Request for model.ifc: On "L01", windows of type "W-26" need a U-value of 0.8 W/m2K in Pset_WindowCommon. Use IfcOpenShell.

First a look at what the model holds.

```python
import ifcopenshell
import ifcopenshell.util.element

model = ifcopenshell.open("model.ifc")
print(model.schema)
storey = next(s for s in model.by_type("IfcBuildingStorey") if s.Name == "L01")
windows = [e for e in ifcopenshell.util.element.get_decomposition(storey) if e.is_a("IfcWindow")]
seen = {}
for e in windows:
    element_type = ifcopenshell.util.element.get_type(e)
    key = (element_type.Name if element_type != e and element_type else None, ifcopenshell.util.element.get_pset(e, "Pset_WindowCommon", "ThermalTransmittance"))
    seen[key] = seen.get(key, 0) + 1
for (name, value), count in sorted(seen.items(), key=str):
    print(count, "x", name, "|", value)
```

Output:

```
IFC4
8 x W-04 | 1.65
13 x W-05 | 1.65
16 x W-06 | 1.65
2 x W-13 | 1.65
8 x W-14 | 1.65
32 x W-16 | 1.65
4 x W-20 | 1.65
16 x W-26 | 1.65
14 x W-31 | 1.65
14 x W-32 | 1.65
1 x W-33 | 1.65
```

```python
import ifcopenshell
import ifcopenshell.api.pset
import ifcopenshell.util.element

model = ifcopenshell.open("model.ifc")

storey = next(s for s in model.by_type("IfcBuildingStorey") if s.Name == "L01")
windows = [e for e in ifcopenshell.util.element.get_decomposition(storey) if e.is_a("IfcWindow")]

count = 0
for e in windows:
    element_type = ifcopenshell.util.element.get_type(e)
    if element_type in (None, e) or element_type.Name != "W-26":
        continue
    # add_pset returns the element's existing set when there is one.
    pset = ifcopenshell.api.pset.add_pset(model, product=e, name="Pset_WindowCommon")
    ifcopenshell.api.pset.edit_pset(model, pset=pset, properties={"ThermalTransmittance": 0.8})
    count += 1

print(count, "windows updated")

model.write("model_edited.ifc")
```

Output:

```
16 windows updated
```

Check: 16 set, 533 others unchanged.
